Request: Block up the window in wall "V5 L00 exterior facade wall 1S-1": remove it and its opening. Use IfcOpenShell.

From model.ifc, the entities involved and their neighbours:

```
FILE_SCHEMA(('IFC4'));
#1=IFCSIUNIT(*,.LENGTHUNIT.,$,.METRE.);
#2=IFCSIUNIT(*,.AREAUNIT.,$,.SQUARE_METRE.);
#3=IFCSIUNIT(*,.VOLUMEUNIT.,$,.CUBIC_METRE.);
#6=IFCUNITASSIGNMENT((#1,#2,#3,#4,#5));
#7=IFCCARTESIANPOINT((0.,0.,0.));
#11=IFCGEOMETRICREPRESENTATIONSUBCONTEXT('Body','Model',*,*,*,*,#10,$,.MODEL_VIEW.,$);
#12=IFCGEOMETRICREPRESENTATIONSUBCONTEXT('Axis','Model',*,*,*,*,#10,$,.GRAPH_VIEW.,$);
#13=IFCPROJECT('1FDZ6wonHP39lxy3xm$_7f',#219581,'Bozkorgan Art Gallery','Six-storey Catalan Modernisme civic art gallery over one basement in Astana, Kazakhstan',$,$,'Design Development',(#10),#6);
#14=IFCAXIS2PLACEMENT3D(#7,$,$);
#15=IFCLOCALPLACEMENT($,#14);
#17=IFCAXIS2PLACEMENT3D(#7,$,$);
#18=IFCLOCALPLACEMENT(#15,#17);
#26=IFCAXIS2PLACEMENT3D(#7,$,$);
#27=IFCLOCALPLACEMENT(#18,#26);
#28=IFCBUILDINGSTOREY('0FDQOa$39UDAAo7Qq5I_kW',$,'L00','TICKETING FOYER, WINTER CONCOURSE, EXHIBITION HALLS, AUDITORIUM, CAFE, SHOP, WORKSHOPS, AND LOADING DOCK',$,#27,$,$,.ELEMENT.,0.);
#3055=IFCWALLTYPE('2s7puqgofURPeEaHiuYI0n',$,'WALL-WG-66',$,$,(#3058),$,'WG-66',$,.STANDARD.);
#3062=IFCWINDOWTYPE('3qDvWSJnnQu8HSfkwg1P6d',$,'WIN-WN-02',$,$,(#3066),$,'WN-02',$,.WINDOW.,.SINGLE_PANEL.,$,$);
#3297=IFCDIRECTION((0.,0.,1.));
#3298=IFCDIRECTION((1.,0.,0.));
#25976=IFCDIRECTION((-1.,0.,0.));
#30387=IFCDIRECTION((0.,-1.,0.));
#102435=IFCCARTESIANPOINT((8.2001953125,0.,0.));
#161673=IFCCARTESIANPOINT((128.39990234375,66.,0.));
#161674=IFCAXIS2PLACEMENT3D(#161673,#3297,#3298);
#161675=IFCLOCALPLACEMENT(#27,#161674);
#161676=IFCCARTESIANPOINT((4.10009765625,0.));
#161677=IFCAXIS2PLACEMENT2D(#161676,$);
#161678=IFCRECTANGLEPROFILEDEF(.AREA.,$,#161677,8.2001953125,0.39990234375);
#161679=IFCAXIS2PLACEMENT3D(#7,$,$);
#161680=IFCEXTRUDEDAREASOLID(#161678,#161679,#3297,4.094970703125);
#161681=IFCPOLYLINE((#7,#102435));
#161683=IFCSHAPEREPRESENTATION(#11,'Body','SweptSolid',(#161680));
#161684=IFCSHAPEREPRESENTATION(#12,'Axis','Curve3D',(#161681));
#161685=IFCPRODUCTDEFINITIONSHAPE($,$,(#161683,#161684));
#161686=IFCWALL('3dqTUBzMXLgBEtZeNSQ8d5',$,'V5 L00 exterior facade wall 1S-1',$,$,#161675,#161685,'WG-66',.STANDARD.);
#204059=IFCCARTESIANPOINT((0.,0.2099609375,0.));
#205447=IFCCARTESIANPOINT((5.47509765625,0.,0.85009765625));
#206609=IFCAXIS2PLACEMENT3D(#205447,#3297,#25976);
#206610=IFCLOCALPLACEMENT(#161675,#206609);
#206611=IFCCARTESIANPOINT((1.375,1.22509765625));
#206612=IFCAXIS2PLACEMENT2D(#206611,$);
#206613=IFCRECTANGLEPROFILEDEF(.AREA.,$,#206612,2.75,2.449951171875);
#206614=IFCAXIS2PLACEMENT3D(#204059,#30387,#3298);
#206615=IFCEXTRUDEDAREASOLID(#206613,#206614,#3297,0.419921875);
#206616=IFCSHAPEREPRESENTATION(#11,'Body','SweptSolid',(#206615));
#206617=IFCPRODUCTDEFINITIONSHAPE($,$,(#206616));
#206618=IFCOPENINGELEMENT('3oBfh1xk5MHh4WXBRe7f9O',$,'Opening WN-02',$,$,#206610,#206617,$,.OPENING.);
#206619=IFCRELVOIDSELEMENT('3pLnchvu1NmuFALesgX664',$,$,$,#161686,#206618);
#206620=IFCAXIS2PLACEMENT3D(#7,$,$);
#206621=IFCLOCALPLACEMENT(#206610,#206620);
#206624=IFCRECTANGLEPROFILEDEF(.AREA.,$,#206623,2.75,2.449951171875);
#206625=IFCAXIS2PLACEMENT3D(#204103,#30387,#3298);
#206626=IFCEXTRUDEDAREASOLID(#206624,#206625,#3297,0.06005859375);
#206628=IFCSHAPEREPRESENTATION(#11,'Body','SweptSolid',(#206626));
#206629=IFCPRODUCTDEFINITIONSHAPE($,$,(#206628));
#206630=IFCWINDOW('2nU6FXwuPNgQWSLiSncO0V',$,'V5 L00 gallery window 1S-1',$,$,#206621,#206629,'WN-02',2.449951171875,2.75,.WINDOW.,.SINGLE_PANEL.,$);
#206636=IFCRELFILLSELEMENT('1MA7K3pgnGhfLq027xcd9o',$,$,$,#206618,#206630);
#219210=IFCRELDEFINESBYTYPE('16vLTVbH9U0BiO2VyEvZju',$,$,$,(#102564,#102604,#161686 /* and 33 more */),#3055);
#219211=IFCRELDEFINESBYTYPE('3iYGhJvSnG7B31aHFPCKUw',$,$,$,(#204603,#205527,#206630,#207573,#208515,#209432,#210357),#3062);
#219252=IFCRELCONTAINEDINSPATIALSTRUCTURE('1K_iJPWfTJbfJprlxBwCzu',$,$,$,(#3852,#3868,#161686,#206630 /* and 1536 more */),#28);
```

```python
import ifcopenshell
import ifcopenshell.api.feature
import ifcopenshell.api.root
import ifcopenshell.geom
import ifcopenshell.util.shape

model = ifcopenshell.open("model.ifc")
settings = ifcopenshell.geom.settings()


def volume(element):
    """Net volume in cubic metres, openings subtracted."""
    shape = ifcopenshell.geom.create_shape(settings, element)
    return ifcopenshell.util.shape.get_volume(shape.geometry)


window = model.by_guid("2nU6FXwuPNgQWSLiSncO0V")
opening = window.FillsVoids[0].RelatingOpeningElement
wall = opening.VoidsElements[0].RelatingBuildingElement
before = volume(wall)

ifcopenshell.api.root.remove_product(model, product=window)
ifcopenshell.api.feature.remove_feature(model, feature=opening)

after = volume(wall)

print(f"wall volume {before:.3f} -> {after:.3f} m3")

model.write("model_v2.ifc")
```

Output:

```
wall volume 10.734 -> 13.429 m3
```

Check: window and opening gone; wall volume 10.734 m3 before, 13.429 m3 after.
